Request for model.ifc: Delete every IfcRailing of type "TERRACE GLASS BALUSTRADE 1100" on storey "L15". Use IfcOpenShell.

First a look at what the model holds.

```python
import ifcopenshell
import ifcopenshell.util.element

model = ifcopenshell.open("model.ifc")
print(model.schema)
storey = next(s for s in model.by_type("IfcBuildingStorey") if s.Name == "L15")
railings = [e for e in ifcopenshell.util.element.get_decomposition(storey) if e.is_a("IfcRailing")]
seen = {}
for e in railings:
    element_type = ifcopenshell.util.element.get_type(e)
    name = element_type.Name if element_type not in (None, e) else None
    seen[name] = seen.get(name, 0) + 1
for name, count in sorted(seen.items(), key=str):
    print(count, "x", name)
```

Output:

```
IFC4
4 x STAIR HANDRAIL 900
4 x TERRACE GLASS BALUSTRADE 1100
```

```python
import ifcopenshell
import ifcopenshell.api.root
import ifcopenshell.util.element

model = ifcopenshell.open("model.ifc")

storey = next(s for s in model.by_type("IfcBuildingStorey") if s.Name == "L15")
railings = [e for e in ifcopenshell.util.element.get_decomposition(storey) if e.is_a("IfcRailing")]
targets = [e for e in railings if (t := ifcopenshell.util.element.get_type(e)) not in (None, e) and t.Name == "TERRACE GLASS BALUSTRADE 1100"]

for e in targets:
    ifcopenshell.api.root.remove_product(model, product=e)
print(len(targets), "removed")

model.write("model_edited.ifc")
```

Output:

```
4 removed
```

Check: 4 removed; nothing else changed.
